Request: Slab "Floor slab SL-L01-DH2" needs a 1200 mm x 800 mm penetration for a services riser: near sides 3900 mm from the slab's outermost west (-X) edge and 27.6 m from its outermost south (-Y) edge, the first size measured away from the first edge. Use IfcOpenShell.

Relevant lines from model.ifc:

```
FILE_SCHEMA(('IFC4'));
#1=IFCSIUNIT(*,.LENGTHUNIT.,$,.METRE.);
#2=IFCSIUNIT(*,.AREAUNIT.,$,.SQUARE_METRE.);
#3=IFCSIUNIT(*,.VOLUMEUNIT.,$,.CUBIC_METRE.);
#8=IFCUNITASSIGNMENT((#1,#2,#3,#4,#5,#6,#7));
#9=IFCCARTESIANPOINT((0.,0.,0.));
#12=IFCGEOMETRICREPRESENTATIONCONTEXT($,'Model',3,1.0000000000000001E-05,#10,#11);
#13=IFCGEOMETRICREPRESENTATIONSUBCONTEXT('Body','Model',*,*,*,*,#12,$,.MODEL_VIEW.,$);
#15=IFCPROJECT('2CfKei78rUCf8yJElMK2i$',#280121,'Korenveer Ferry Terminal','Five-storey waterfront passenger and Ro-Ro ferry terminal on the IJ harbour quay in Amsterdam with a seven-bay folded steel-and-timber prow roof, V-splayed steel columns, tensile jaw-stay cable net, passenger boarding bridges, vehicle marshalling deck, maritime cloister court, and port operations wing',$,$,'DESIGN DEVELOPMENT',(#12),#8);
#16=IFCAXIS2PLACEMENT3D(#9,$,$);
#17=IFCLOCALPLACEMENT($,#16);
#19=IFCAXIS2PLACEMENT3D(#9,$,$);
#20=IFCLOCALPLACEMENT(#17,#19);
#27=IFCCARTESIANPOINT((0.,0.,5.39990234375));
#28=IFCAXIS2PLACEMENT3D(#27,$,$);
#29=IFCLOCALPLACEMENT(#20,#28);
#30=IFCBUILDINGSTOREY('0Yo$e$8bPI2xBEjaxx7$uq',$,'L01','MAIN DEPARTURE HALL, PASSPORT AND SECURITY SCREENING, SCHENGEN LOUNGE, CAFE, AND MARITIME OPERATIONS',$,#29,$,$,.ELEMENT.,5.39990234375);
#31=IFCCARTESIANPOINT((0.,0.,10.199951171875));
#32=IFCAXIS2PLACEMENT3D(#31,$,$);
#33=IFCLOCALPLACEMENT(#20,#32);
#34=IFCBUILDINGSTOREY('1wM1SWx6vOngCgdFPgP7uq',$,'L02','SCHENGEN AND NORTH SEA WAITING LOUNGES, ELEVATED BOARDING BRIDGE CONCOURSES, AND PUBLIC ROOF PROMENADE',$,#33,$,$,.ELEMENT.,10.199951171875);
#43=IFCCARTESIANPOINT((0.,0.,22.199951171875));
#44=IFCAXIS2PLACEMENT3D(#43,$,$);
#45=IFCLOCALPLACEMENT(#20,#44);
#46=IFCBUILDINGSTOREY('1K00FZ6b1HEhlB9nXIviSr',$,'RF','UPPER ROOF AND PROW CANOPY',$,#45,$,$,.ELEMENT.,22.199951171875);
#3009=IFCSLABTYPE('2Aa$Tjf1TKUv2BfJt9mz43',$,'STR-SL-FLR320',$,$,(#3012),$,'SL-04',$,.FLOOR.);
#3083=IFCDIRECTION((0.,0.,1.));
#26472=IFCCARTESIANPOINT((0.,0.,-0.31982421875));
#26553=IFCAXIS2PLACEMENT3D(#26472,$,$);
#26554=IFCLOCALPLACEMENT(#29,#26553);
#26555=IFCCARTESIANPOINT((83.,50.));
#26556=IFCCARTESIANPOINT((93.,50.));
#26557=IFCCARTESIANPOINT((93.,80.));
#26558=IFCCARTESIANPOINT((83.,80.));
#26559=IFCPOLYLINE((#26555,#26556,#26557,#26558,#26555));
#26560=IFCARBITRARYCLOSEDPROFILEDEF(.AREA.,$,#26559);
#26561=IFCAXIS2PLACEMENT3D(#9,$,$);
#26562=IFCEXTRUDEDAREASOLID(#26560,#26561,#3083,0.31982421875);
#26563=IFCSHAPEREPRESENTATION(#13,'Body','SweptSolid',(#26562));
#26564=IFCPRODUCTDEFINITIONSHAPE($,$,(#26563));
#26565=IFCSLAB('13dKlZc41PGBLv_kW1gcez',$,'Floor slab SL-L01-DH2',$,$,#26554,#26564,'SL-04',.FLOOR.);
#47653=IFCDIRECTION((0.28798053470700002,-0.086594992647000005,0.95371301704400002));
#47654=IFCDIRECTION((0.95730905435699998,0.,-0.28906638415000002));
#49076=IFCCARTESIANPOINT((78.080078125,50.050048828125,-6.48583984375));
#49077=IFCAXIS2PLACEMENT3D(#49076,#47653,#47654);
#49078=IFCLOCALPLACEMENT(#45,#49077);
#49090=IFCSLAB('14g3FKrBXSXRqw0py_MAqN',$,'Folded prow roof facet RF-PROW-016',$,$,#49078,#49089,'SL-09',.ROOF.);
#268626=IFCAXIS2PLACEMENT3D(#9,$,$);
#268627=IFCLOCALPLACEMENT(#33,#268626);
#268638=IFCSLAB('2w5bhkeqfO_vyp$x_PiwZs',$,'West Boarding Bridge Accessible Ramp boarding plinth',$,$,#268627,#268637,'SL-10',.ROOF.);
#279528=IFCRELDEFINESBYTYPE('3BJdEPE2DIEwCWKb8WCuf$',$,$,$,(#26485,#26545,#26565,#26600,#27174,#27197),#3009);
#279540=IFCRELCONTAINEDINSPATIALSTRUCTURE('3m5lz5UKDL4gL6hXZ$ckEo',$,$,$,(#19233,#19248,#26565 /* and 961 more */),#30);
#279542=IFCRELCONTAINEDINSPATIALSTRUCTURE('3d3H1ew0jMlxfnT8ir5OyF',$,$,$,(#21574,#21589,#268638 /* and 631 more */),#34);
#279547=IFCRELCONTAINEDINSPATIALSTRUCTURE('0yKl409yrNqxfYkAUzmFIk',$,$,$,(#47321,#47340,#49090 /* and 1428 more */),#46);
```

```python
import numpy as np
import ifcopenshell
import ifcopenshell.api.feature
import ifcopenshell.api.geometry
import ifcopenshell.api.root
import ifcopenshell.geom
import ifcopenshell.util.placement
import ifcopenshell.util.representation
import ifcopenshell.util.shape
import ifcopenshell.util.unit

model = ifcopenshell.open("model.ifc")
unit_scale = ifcopenshell.util.unit.calculate_unit_scale(model)
settings = ifcopenshell.geom.settings()


def volume(element):
    """Net volume in cubic metres, openings subtracted."""
    shape = ifcopenshell.geom.create_shape(settings, element)
    return ifcopenshell.util.shape.get_volume(shape.geometry)


slab = model.by_id(26565)
before = volume(slab)

# Extent in the slab's own axes, in metres. The edges named are its -X and -Y sides.
slab_shape = ifcopenshell.geom.create_shape(settings, slab)
vertices = ifcopenshell.util.shape.get_vertices(slab_shape.geometry)
x_min, y_min, bottom = vertices.min(axis=0)
top = vertices[:, 2].max()

opening = ifcopenshell.api.root.create_entity(model, ifc_class="IfcOpeningElement", name="Services riser opening", predefined_type="OPENING")
context = ifcopenshell.util.representation.get_context(model, "Model", "Body", "MODEL_VIEW")
width, depth = 1.2, 0.8
outline = [(0.0, 0.0), (width, 0.0), (width, depth), (0.0, depth), (0.0, 0.0)]
# Overshoot both faces by 50 mm so the cut is clean.
shape = ifcopenshell.api.geometry.add_slab_representation(
    model, context=context, depth=top - bottom + 0.1, polyline=outline
)
ifcopenshell.api.geometry.assign_representation(model, product=opening, representation=shape)

matrix = ifcopenshell.util.placement.get_local_placement(slab.ObjectPlacement)
matrix[:, 3] = matrix @ np.append(np.array([x_min + 3.9, y_min + 27.6, bottom - 0.05]) / unit_scale, 1.0)
ifcopenshell.api.geometry.edit_object_placement(model, product=opening, matrix=matrix, is_si=False)
ifcopenshell.api.feature.add_feature(model, feature=opening, element=slab)

after = volume(slab)

print(f"slab volume {before:.3f} -> {after:.3f} m3")

model.write("model_rev.ifc")
```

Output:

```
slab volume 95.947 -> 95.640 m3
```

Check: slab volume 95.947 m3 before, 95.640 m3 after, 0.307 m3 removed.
